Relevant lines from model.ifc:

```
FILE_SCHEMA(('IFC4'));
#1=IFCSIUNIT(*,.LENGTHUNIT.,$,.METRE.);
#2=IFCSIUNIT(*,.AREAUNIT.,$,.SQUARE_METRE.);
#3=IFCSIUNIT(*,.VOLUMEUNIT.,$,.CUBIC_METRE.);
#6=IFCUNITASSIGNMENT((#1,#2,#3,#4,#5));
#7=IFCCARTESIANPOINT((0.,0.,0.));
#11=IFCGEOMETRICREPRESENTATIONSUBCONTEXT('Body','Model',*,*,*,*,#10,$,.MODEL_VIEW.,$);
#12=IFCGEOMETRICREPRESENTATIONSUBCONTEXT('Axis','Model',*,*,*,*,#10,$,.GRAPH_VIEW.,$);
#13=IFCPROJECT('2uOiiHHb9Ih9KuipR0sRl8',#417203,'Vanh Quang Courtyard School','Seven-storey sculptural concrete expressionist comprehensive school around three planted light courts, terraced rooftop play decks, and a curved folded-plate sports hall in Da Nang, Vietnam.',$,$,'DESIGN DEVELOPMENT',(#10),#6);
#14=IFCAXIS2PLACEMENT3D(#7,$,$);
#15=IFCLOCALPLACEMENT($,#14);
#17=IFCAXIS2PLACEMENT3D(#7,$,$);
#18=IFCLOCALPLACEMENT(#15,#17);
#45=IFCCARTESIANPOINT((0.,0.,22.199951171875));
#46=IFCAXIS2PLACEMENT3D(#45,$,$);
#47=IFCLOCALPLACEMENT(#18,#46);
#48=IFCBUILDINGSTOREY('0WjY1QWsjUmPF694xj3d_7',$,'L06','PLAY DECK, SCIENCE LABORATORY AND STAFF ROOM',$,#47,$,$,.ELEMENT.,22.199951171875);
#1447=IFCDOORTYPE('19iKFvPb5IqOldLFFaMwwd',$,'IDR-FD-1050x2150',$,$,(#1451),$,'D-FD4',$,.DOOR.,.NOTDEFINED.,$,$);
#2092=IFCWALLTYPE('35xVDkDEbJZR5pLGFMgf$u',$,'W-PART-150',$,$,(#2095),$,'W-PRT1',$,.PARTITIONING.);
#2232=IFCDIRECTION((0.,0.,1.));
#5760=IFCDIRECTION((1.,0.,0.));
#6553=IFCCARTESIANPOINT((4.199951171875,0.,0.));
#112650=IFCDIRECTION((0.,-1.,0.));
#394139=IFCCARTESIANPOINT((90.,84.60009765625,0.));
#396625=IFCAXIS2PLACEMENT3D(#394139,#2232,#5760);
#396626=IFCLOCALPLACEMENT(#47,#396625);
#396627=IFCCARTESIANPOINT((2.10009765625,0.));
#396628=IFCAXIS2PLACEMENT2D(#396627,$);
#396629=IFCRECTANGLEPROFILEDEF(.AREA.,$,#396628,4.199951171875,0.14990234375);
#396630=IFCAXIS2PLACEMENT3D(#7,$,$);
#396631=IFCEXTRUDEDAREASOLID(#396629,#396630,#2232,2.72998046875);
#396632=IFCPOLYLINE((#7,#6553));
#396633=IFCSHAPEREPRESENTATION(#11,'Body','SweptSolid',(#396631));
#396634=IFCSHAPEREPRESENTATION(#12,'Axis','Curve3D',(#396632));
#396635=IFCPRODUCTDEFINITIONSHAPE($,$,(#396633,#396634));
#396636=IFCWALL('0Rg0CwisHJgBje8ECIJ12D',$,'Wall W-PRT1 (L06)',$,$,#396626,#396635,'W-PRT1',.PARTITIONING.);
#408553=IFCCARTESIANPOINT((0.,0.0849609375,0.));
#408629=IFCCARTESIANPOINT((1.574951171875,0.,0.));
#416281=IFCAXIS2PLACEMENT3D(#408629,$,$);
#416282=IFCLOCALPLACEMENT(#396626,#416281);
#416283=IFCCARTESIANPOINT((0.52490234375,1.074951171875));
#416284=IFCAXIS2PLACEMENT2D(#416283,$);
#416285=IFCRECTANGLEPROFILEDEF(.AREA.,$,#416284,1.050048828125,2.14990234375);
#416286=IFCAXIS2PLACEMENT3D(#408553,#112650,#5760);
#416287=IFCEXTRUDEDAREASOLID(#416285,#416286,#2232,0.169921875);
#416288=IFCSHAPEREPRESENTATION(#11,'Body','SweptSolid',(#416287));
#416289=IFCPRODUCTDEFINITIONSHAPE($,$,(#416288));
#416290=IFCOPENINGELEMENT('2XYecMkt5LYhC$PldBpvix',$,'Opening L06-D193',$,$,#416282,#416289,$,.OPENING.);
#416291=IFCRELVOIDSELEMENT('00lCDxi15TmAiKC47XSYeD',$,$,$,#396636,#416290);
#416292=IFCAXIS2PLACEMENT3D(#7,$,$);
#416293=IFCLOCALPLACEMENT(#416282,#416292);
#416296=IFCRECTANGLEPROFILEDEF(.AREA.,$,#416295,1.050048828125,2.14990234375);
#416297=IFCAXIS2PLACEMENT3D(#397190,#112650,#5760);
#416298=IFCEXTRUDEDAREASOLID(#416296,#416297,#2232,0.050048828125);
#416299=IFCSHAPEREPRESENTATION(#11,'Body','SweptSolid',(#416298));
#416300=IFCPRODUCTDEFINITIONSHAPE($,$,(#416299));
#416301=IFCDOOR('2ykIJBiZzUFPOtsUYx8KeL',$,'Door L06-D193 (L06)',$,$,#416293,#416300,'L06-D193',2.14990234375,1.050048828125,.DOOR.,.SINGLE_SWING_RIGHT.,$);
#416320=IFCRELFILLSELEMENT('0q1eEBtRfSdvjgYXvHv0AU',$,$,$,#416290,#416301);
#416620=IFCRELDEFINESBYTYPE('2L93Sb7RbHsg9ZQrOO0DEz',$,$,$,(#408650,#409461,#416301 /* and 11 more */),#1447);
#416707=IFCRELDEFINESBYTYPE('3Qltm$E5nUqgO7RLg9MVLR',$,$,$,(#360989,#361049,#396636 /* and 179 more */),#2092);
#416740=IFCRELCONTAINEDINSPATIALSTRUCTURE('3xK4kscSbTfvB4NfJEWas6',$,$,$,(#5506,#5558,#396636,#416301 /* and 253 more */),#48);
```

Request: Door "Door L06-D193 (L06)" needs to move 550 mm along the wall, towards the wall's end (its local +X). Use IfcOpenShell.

```python
import ifcopenshell
import ifcopenshell.api.geometry
import ifcopenshell.util.placement
import ifcopenshell.util.unit

model = ifcopenshell.open("model.ifc")
unit_scale = ifcopenshell.util.unit.calculate_unit_scale(model)

door = model.by_id(416301)
opening = door.FillsVoids[0].RelatingOpeningElement
wall = opening.VoidsElements[0].RelatingBuildingElement

wall_matrix = ifcopenshell.util.placement.get_local_placement(wall.ObjectPlacement)
shift = wall_matrix[:3, 0] * 0.55 / unit_scale
before = ifcopenshell.util.placement.get_local_placement(door.ObjectPlacement)[:3, 3].copy()

# The door is placed relative to its opening, so it follows when the opening moves.
matrix = ifcopenshell.util.placement.get_local_placement(opening.ObjectPlacement)
matrix[:3, 3] += shift
ifcopenshell.api.geometry.edit_object_placement(
    model, product=opening, matrix=matrix, is_si=False, should_transform_children=True
)

after = ifcopenshell.util.placement.get_local_placement(door.ObjectPlacement)[:3, 3]
print("door moved by", (after - before).round(3) + 0.0)

model.write("model-out.ifc")
```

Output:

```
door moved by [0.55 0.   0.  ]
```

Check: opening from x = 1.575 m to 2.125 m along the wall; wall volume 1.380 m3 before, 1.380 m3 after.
